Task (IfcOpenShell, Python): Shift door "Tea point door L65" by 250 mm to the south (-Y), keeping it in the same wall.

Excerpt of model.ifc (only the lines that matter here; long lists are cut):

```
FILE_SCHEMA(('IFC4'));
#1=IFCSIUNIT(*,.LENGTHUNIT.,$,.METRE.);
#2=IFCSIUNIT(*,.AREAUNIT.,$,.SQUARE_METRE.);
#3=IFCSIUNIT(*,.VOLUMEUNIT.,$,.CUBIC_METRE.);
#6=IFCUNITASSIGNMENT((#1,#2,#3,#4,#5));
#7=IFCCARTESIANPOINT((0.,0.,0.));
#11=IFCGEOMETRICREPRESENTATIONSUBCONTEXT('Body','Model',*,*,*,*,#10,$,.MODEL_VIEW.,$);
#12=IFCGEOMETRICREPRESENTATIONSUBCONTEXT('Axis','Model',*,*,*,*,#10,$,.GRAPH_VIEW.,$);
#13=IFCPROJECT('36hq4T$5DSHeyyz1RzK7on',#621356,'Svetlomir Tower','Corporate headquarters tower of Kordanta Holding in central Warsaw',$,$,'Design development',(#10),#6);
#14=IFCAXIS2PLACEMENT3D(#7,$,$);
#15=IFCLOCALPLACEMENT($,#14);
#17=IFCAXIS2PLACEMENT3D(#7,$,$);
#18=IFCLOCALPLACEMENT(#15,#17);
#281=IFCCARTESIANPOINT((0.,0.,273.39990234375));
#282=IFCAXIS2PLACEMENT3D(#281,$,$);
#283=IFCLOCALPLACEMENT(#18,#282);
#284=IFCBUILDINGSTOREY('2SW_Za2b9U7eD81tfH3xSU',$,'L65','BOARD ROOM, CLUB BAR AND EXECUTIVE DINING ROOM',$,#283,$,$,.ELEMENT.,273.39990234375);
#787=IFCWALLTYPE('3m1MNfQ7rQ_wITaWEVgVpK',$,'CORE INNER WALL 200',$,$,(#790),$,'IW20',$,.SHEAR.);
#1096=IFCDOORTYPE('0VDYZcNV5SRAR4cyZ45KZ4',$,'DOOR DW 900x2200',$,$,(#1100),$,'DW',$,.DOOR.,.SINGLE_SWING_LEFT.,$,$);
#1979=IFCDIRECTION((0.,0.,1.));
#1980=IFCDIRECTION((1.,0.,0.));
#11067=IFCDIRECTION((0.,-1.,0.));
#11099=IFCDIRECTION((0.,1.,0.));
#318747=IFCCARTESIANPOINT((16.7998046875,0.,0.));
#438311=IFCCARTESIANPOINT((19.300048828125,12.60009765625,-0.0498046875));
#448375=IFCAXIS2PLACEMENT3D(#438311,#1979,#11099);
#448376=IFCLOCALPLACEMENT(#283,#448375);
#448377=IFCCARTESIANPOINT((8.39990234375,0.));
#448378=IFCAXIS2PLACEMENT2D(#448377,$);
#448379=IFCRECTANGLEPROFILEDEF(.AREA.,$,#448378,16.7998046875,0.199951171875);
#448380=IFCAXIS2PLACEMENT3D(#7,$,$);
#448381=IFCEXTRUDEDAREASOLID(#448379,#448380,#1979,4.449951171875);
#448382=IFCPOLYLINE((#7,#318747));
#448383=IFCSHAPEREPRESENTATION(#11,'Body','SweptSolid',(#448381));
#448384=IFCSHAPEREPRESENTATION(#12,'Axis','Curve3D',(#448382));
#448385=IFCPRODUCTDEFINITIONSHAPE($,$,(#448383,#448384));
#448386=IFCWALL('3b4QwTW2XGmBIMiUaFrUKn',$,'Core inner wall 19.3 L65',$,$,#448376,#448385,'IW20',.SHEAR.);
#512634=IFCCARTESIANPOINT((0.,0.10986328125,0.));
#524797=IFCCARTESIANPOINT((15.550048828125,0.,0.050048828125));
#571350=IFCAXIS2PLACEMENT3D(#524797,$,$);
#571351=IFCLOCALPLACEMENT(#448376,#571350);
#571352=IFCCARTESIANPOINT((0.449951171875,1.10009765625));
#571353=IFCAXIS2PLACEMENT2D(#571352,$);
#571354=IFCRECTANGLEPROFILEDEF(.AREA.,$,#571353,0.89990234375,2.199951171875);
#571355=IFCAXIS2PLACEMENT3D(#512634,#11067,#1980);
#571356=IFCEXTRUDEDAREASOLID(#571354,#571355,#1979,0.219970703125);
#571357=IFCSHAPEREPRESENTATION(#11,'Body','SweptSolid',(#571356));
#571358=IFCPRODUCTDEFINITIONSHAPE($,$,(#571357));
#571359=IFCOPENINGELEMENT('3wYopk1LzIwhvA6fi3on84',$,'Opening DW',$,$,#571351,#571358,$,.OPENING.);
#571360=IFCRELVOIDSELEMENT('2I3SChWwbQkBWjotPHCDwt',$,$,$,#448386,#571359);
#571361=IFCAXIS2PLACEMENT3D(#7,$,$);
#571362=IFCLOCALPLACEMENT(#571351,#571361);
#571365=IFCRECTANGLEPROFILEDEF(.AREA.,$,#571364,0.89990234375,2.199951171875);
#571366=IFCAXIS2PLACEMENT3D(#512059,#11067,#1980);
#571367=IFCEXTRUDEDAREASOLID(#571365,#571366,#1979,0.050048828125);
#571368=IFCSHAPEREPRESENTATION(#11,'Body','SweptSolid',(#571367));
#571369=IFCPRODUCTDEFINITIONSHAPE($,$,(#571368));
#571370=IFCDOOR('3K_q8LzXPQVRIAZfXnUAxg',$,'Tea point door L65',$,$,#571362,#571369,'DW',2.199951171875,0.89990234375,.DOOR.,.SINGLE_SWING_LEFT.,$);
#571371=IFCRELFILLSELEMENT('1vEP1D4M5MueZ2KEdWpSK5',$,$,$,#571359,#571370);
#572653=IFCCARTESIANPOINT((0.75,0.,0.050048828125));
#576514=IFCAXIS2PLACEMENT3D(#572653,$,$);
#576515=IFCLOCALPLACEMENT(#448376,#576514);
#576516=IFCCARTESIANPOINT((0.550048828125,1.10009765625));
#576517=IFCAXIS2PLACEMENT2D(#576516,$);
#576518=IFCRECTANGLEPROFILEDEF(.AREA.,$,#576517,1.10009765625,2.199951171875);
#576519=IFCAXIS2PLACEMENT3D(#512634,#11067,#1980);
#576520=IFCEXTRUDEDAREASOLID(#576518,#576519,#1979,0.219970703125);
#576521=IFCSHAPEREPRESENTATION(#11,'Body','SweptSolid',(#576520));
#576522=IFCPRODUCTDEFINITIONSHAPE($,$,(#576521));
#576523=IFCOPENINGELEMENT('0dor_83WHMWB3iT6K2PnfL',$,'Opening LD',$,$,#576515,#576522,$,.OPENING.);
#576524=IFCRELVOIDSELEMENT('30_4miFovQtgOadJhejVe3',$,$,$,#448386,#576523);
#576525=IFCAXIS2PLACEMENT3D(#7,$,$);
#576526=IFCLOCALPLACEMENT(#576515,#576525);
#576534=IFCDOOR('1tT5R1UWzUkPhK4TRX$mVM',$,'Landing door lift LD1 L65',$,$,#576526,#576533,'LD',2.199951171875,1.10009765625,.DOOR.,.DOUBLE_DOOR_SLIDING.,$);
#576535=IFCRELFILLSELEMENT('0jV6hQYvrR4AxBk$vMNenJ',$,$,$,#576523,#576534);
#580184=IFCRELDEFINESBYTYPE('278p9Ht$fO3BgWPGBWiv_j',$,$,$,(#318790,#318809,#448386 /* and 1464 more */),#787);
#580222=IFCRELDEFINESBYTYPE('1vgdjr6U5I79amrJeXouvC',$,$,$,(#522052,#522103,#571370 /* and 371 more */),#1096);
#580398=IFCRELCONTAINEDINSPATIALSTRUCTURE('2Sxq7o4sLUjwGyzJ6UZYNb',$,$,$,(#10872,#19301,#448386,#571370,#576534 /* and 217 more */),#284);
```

```python
import ifcopenshell
import ifcopenshell.api.geometry
import ifcopenshell.util.placement
import ifcopenshell.util.unit

model = ifcopenshell.open("model.ifc")
unit_scale = ifcopenshell.util.unit.calculate_unit_scale(model)

door = model.by_guid("3K_q8LzXPQVRIAZfXnUAxg")
opening = door.FillsVoids[0].RelatingOpeningElement
wall = opening.VoidsElements[0].RelatingBuildingElement

wall_matrix = ifcopenshell.util.placement.get_local_placement(wall.ObjectPlacement)
shift = wall_matrix[:3, 0] * -0.25 / unit_scale
before = ifcopenshell.util.placement.get_local_placement(door.ObjectPlacement)[:3, 3].copy()

# The door is placed relative to its opening, so it follows when the opening moves.
matrix = ifcopenshell.util.placement.get_local_placement(opening.ObjectPlacement)
matrix[:3, 3] += shift
ifcopenshell.api.geometry.edit_object_placement(
    model, product=opening, matrix=matrix, is_si=False, should_transform_children=True
)

after = ifcopenshell.util.placement.get_local_placement(door.ObjectPlacement)[:3, 3]
print("door moved by", (after - before).round(3) + 0.0)

model.write("model_updated.ifc")
```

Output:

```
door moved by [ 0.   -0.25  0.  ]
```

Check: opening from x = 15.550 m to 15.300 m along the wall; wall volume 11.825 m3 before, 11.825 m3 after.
